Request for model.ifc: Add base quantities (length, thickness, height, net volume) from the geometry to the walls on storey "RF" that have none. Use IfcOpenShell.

First a look at what the model holds.

```python
import ifcopenshell
import ifcopenshell.util.element
import ifcopenshell.util.unit

model = ifcopenshell.open("model.ifc")
print(model.schema)
for unit_type in ("LENGTHUNIT", "AREAUNIT", "VOLUMEUNIT"):
    print(unit_type, ifcopenshell.util.unit.calculate_unit_scale(model, unit_type))
storey = next(s for s in model.by_type("IfcBuildingStorey") if s.Name == "RF")
walls = [e for e in ifcopenshell.util.element.get_decomposition(storey) if e.is_a("IfcWall")]
for e in sorted(walls, key=lambda e: e.id()):
    print(e.id(), e.is_a(), e.Name, list(ifcopenshell.util.element.get_psets(e, qtos_only=True)), sep=" | ")
```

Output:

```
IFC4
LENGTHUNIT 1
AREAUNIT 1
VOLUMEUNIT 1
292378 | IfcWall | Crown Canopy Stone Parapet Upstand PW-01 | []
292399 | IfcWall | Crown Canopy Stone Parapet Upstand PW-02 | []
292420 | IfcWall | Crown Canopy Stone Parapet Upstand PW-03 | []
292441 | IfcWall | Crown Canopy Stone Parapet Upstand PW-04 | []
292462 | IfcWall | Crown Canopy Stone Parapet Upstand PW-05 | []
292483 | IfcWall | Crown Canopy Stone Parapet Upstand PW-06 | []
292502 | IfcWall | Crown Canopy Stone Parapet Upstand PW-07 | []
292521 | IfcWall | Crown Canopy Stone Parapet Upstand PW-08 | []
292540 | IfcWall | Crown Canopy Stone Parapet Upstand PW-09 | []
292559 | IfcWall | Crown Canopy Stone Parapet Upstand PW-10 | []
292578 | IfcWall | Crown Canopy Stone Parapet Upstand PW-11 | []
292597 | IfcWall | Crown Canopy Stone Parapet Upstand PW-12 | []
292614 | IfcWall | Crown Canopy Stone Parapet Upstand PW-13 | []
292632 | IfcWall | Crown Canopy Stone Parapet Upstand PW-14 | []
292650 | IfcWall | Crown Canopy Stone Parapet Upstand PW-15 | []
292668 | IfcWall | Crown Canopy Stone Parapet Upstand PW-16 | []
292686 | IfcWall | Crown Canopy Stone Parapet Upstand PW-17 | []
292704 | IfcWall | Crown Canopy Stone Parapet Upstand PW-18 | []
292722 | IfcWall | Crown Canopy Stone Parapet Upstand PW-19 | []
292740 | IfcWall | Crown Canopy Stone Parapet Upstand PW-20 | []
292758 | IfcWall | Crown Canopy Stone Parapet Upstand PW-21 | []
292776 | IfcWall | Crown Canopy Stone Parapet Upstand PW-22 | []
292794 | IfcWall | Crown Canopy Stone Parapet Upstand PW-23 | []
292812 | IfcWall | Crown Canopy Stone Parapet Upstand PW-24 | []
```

```python
import ifcopenshell
import ifcopenshell.api.pset
import ifcopenshell.geom
import ifcopenshell.util.element
import ifcopenshell.util.shape
import ifcopenshell.util.unit

model = ifcopenshell.open("model.ifc")
unit_scale = ifcopenshell.util.unit.calculate_unit_scale(model)
volume_scale = ifcopenshell.util.unit.calculate_unit_scale(model, "VOLUMEUNIT")
settings = ifcopenshell.geom.settings()

storey = next(s for s in model.by_type("IfcBuildingStorey") if s.Name == "RF")
walls = [e for e in ifcopenshell.util.element.get_decomposition(storey) if e.is_a("IfcWall")]

for e in sorted(walls, key=lambda e: e.id()):
    if ifcopenshell.util.element.get_psets(e, qtos_only=True, should_inherit=False):
        continue
    # Geometry comes back in metres, in the element's own axes.
    shape = ifcopenshell.geom.create_shape(settings, e)
    values = {
        "Length": ifcopenshell.util.shape.get_x(shape.geometry) / unit_scale,
        "Width": ifcopenshell.util.shape.get_y(shape.geometry) / unit_scale,
        "Height": ifcopenshell.util.shape.get_z(shape.geometry) / unit_scale,
        "NetVolume": ifcopenshell.util.shape.get_volume(shape.geometry) / volume_scale,
    }
    qto = ifcopenshell.api.pset.add_qto(model, product=e, name="Qto_WallBaseQuantities")
    ifcopenshell.api.pset.edit_qto(model, qto=qto, properties=values)
    print(e.id(), {k: round(v, 3) for k, v in values.items()})

model.write("model-out.ifc")
```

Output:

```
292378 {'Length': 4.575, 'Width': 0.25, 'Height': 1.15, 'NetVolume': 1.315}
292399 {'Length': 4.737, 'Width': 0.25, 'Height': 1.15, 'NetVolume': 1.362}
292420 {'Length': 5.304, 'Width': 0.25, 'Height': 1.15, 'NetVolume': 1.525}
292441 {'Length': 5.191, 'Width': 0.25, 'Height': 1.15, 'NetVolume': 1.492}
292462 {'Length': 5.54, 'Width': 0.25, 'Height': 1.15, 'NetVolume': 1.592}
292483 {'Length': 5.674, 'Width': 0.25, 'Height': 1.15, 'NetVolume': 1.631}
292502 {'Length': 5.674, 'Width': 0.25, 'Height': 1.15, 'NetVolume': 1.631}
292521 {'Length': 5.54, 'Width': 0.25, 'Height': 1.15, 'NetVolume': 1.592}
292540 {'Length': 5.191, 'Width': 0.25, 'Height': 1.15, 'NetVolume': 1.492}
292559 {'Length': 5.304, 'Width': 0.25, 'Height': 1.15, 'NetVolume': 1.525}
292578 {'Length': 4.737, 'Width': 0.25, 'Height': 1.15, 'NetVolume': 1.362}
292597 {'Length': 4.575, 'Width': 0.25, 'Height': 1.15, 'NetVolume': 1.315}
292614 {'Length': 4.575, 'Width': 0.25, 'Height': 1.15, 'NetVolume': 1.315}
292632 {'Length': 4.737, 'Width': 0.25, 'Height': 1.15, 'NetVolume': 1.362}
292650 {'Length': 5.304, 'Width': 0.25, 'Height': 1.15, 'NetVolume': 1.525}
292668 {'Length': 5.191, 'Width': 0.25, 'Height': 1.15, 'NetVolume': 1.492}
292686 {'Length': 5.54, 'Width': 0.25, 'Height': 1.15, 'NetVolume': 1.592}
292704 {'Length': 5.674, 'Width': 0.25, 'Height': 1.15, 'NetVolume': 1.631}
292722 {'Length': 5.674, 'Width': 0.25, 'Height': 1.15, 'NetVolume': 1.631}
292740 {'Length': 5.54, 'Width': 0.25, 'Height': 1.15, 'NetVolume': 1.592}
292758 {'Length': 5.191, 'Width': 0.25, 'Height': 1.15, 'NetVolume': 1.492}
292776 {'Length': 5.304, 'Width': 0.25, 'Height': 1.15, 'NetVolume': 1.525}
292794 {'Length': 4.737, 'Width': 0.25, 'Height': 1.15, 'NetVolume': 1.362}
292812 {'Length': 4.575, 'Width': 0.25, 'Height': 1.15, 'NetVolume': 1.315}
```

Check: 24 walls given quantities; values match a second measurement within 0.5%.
